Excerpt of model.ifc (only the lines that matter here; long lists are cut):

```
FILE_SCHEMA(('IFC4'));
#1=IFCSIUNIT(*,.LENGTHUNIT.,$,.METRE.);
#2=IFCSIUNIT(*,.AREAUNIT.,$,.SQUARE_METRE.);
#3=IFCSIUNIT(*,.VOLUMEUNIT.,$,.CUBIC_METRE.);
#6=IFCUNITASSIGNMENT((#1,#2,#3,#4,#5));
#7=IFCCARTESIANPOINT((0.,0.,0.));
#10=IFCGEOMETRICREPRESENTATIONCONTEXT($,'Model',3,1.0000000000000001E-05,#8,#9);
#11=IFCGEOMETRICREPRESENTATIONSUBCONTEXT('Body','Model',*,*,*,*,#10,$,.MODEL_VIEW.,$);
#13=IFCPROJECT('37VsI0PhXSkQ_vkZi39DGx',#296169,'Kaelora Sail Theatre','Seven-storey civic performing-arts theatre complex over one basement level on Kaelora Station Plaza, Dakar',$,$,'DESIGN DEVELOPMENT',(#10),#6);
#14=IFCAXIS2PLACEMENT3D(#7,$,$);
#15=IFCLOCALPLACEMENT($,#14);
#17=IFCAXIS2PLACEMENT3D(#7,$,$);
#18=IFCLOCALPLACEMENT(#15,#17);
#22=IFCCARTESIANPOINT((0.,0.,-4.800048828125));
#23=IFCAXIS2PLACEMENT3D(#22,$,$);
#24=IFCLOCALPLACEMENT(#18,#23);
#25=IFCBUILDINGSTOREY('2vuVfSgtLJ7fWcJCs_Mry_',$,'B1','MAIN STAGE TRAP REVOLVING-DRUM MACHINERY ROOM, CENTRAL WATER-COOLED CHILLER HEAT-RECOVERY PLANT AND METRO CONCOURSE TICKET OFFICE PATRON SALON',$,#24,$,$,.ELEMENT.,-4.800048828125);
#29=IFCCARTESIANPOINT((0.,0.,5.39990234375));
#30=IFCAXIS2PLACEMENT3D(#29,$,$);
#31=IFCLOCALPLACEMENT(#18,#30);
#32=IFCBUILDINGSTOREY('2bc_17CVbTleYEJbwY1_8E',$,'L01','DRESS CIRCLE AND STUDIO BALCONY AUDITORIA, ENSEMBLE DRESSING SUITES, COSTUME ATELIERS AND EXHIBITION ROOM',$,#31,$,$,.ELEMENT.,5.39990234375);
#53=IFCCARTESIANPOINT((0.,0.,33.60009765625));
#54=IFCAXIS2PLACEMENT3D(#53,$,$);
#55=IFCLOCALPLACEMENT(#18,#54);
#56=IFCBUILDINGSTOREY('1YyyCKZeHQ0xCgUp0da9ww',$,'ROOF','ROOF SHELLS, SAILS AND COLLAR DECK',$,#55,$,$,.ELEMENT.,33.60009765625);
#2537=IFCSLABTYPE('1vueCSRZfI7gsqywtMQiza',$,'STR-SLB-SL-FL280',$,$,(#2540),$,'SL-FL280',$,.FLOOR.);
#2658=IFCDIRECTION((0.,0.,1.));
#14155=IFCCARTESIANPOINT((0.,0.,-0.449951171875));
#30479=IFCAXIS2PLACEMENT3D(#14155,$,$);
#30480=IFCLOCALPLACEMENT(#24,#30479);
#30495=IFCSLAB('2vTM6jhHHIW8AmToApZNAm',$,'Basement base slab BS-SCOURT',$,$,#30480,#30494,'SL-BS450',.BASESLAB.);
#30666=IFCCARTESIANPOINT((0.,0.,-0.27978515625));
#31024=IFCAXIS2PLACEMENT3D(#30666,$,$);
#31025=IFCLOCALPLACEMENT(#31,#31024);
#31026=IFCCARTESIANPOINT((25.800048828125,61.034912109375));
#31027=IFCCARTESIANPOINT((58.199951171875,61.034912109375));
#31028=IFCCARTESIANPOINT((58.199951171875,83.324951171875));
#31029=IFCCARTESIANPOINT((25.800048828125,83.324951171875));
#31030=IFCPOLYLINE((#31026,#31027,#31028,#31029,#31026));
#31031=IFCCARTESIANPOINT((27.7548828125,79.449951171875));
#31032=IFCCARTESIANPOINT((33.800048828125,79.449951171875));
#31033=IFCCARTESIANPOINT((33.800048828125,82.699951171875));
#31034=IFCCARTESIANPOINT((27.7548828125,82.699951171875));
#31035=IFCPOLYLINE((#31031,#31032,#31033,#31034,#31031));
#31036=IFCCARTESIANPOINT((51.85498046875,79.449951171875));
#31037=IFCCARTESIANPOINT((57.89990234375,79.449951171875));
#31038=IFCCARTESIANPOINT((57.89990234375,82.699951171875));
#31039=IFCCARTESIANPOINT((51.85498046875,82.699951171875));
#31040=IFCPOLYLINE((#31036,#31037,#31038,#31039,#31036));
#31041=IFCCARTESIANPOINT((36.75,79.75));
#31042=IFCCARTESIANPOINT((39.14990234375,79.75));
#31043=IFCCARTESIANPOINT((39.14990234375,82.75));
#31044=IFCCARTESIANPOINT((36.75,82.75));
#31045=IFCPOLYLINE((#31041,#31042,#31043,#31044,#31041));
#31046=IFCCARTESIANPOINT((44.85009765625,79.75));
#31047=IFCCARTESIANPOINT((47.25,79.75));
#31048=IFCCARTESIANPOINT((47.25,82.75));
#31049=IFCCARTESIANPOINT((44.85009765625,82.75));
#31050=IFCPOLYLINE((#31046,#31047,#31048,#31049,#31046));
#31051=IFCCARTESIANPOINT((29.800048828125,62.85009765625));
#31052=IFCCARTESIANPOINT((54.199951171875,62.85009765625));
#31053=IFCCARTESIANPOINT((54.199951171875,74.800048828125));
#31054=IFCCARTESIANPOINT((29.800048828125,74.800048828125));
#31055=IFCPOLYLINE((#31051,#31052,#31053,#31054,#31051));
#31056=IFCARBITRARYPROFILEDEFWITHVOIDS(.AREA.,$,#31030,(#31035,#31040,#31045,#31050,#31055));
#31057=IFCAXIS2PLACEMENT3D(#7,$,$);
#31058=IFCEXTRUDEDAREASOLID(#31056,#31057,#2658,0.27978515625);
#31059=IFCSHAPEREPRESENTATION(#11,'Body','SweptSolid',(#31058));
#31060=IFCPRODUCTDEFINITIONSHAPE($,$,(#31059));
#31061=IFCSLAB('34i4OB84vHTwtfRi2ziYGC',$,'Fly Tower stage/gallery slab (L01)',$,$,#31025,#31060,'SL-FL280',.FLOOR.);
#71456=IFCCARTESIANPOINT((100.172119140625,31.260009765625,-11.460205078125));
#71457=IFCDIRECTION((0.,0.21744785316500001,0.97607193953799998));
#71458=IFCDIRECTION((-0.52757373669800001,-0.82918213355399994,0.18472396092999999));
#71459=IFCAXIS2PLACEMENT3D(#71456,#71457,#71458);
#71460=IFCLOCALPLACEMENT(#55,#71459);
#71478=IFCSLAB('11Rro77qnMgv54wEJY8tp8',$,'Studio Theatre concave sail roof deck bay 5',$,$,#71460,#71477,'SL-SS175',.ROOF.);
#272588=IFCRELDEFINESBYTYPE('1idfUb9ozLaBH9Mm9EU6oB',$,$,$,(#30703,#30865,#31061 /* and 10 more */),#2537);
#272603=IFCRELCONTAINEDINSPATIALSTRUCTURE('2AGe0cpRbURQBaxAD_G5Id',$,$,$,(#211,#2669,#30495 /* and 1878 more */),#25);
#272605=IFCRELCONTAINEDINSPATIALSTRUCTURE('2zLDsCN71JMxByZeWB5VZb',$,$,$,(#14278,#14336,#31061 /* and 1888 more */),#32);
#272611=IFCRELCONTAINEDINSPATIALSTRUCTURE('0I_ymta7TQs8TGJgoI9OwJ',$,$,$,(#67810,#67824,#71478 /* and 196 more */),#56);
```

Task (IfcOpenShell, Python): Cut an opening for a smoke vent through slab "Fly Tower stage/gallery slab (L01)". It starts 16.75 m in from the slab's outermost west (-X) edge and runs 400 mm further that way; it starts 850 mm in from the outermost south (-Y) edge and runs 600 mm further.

```python
import numpy as np
import ifcopenshell
import ifcopenshell.api.feature
import ifcopenshell.api.geometry
import ifcopenshell.api.root
import ifcopenshell.geom
import ifcopenshell.util.placement
import ifcopenshell.util.representation
import ifcopenshell.util.shape
import ifcopenshell.util.unit

model = ifcopenshell.open("model.ifc")
unit_scale = ifcopenshell.util.unit.calculate_unit_scale(model)
settings = ifcopenshell.geom.settings()


def volume(element):
    """Net volume in cubic metres, openings subtracted."""
    shape = ifcopenshell.geom.create_shape(settings, element)
    return ifcopenshell.util.shape.get_volume(shape.geometry)


slab = model.by_id(31061)
before = volume(slab)

# Extent in the slab's own axes, in metres. The edges named are its -X and -Y sides.
slab_shape = ifcopenshell.geom.create_shape(settings, slab)
vertices = ifcopenshell.util.shape.get_vertices(slab_shape.geometry)
x_min, y_min, bottom = vertices.min(axis=0)
top = vertices[:, 2].max()

opening = ifcopenshell.api.root.create_entity(model, ifc_class="IfcOpeningElement", name="Smoke vent opening", predefined_type="OPENING")
context = ifcopenshell.util.representation.get_context(model, "Model", "Body", "MODEL_VIEW")
width, depth = 0.4, 0.6
outline = [(0.0, 0.0), (width, 0.0), (width, depth), (0.0, depth), (0.0, 0.0)]
# Overshoot both faces by 50 mm so the cut is clean.
shape = ifcopenshell.api.geometry.add_slab_representation(
    model, context=context, depth=top - bottom + 0.1, polyline=outline
)
ifcopenshell.api.geometry.assign_representation(model, product=opening, representation=shape)

matrix = ifcopenshell.util.placement.get_local_placement(slab.ObjectPlacement)
matrix[:, 3] = matrix @ np.append(np.array([x_min + 16.75, y_min + 0.85, bottom - 0.05]) / unit_scale, 1.0)
ifcopenshell.api.geometry.edit_object_placement(model, product=opening, matrix=matrix, is_si=False)
ifcopenshell.api.feature.add_feature(model, feature=opening, element=slab)

after = volume(slab)

print(f"slab volume {before:.3f} -> {after:.3f} m3")

model.write("model_v2.ifc")
```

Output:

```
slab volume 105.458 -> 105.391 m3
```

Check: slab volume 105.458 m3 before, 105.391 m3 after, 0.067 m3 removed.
